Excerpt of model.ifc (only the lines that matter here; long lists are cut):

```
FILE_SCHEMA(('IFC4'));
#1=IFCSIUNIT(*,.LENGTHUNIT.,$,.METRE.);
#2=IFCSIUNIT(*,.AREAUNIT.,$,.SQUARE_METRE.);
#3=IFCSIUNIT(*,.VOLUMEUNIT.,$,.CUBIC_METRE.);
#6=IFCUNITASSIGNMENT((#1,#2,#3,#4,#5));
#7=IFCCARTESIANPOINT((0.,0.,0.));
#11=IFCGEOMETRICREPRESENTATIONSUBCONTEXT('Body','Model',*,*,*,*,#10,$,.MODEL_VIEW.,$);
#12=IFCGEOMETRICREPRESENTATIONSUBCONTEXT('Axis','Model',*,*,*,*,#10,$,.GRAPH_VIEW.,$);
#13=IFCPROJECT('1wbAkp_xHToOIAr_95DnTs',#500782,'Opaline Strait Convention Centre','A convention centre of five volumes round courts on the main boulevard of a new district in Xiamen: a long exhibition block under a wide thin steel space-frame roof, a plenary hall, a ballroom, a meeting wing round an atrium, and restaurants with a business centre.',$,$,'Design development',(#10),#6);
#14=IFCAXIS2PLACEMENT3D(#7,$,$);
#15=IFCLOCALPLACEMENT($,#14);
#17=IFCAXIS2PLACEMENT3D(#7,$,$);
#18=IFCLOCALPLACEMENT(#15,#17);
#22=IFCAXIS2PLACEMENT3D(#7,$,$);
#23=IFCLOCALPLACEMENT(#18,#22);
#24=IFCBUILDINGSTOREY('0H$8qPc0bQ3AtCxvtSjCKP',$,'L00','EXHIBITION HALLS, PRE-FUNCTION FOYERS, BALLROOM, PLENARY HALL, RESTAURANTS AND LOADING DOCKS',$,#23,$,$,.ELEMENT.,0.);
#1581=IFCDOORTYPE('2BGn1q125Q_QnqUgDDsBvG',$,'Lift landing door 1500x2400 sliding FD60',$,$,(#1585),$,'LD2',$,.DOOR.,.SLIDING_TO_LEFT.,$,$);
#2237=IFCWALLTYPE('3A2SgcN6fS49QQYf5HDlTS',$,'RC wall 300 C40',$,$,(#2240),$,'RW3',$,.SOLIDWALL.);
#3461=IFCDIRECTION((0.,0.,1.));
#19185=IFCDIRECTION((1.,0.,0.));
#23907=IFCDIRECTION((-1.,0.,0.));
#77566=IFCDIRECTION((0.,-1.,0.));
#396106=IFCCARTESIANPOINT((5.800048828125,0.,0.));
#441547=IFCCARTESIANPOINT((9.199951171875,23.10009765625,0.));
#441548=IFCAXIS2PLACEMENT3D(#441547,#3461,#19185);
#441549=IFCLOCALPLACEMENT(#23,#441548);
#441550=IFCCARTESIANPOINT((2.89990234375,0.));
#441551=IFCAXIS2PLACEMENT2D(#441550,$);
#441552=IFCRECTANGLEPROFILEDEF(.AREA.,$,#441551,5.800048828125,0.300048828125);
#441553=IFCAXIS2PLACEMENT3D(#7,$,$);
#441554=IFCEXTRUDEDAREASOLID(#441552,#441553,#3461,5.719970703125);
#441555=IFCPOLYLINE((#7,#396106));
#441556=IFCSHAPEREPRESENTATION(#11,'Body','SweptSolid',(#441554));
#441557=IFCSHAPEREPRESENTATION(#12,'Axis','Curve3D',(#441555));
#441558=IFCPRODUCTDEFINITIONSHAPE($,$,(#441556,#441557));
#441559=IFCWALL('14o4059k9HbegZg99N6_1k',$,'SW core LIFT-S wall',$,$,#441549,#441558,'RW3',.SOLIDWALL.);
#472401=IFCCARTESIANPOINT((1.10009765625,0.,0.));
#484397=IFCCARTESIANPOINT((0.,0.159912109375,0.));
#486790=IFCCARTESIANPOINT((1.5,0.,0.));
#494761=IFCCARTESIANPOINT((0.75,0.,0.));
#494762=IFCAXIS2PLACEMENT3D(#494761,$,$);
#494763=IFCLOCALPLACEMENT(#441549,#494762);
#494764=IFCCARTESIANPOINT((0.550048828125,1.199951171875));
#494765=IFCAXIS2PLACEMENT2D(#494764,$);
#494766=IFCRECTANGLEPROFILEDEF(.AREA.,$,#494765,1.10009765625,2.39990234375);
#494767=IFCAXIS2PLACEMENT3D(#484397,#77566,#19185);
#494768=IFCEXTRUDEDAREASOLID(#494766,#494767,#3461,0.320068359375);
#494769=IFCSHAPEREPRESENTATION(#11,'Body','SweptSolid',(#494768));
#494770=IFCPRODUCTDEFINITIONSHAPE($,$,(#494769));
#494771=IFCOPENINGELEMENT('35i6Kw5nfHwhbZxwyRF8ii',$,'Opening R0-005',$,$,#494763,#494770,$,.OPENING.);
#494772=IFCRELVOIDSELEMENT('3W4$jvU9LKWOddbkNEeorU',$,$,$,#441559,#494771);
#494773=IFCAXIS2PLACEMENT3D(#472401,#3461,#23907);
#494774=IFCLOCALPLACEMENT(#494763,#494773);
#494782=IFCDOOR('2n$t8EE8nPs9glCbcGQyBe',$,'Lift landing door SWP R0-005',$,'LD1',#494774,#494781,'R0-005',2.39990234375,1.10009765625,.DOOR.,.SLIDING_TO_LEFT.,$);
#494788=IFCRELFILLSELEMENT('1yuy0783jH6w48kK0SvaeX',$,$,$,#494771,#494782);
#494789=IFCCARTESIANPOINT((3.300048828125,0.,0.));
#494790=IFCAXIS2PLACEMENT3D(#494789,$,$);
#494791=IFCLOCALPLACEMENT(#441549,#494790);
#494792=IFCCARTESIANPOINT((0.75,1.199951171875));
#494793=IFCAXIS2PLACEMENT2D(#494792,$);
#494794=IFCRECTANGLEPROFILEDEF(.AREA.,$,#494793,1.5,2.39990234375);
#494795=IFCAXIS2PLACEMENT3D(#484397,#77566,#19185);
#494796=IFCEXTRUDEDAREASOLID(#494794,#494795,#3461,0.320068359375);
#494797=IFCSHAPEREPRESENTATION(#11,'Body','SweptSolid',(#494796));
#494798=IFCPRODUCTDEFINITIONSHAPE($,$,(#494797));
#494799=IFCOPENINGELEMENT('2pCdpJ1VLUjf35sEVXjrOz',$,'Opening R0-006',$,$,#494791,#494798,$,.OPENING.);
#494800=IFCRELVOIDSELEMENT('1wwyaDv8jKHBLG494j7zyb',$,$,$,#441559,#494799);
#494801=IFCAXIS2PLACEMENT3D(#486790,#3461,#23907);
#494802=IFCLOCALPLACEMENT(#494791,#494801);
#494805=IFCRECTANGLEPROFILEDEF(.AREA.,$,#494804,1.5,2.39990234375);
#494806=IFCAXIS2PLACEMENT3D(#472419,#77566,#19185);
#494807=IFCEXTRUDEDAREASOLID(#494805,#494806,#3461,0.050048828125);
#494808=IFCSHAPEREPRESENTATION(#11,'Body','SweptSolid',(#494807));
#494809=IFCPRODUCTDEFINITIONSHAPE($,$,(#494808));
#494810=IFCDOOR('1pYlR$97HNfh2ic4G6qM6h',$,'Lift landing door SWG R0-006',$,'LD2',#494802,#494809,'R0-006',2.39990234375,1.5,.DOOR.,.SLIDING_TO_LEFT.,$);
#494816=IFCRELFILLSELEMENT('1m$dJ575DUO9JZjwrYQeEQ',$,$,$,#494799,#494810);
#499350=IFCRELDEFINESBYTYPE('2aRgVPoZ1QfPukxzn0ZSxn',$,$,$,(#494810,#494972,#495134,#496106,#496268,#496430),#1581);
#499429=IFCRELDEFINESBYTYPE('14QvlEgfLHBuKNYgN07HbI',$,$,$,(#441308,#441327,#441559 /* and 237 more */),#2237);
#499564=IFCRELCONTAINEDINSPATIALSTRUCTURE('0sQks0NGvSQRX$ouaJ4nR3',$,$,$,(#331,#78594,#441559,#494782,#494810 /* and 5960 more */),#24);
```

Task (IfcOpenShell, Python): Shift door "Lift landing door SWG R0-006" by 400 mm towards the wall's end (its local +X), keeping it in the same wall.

```python
import ifcopenshell
import ifcopenshell.api.geometry
import ifcopenshell.util.placement

model = ifcopenshell.open("model.ifc")

door = model.by_guid("1pYlR$97HNfh2ic4G6qM6h")
opening = door.FillsVoids[0].RelatingOpeningElement
wall = opening.VoidsElements[0].RelatingBuildingElement

wall_matrix = ifcopenshell.util.placement.get_local_placement(wall.ObjectPlacement)
shift = wall_matrix[:3, 0] * 0.4
before = ifcopenshell.util.placement.get_local_placement(door.ObjectPlacement)[:3, 3].copy()

# The door is placed relative to its opening, so it follows when the opening moves.
matrix = ifcopenshell.util.placement.get_local_placement(opening.ObjectPlacement)
matrix[:3, 3] += shift
ifcopenshell.api.geometry.edit_object_placement(
    model, product=opening, matrix=matrix, is_si=False, should_transform_children=True
)

after = ifcopenshell.util.placement.get_local_placement(door.ObjectPlacement)[:3, 3]
print("door moved by", (after - before).round(3) + 0.0)

model.write("model_v2.ifc")
```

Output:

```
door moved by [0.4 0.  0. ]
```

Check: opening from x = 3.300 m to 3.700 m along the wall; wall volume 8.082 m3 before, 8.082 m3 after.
